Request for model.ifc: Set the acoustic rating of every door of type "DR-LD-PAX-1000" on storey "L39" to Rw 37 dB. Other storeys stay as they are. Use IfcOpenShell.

First a look at what the model holds.

```python
import ifcopenshell
import ifcopenshell.util.element

model = ifcopenshell.open("model.ifc")
print(model.schema)
storey = next(s for s in model.by_type("IfcBuildingStorey") if s.Name == "L39")
doors = [e for e in ifcopenshell.util.element.get_decomposition(storey) if e.is_a("IfcDoor")]
seen = {}
for e in doors:
    element_type = ifcopenshell.util.element.get_type(e)
    key = (element_type.Name if element_type != e and element_type else None, ifcopenshell.util.element.get_pset(e, "Pset_DoorCommon", "AcousticRating"))
    seen[key] = seen.get(key, 0) + 1
for (name, value), count in sorted(seen.items(), key=str):
    print(count, "x", name, "|", value)
```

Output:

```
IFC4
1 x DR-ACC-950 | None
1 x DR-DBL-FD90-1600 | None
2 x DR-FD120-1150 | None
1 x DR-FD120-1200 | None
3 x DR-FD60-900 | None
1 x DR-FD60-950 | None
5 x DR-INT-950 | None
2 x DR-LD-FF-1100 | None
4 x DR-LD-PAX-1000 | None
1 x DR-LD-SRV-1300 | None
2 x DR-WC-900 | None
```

```python
import ifcopenshell
import ifcopenshell.api.pset
import ifcopenshell.util.element

model = ifcopenshell.open("model.ifc")

storey = next(s for s in model.by_type("IfcBuildingStorey") if s.Name == "L39")
doors = [e for e in ifcopenshell.util.element.get_decomposition(storey) if e.is_a("IfcDoor")]

count = 0
for e in doors:
    element_type = ifcopenshell.util.element.get_type(e)
    if element_type in (None, e) or element_type.Name != "DR-LD-PAX-1000":
        continue
    found = ifcopenshell.util.element.get_pset(e, "Pset_DoorCommon", should_inherit=False)
    if found:
        pset = model.by_id(found["id"])
        if len(ifcopenshell.util.element.get_elements_by_pset(pset)) > 1:
            pset = ifcopenshell.api.pset.unshare_pset(model, products=[e], pset=pset)[0]
    else:
        pset = ifcopenshell.api.pset.add_pset(model, product=e, name="Pset_DoorCommon")
    ifcopenshell.api.pset.edit_pset(model, pset=pset, properties={"AcousticRating": "Rw 37 dB"})
    count += 1

print(count, "doors updated")

model.write("model_v2.ifc")
```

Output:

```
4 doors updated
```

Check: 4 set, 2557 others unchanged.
